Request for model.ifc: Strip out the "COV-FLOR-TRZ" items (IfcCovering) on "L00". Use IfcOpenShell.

First a look at what the model holds.

```python
import ifcopenshell
import ifcopenshell.util.element

model = ifcopenshell.open("model.ifc")
print(model.schema)
storey = next(s for s in model.by_type("IfcBuildingStorey") if s.Name == "L00")
coverings = [e for e in ifcopenshell.util.element.get_decomposition(storey) if e.is_a("IfcCovering")]
seen = {}
for e in coverings:
    element_type = ifcopenshell.util.element.get_type(e)
    name = element_type.Name if element_type not in (None, e) else None
    seen[name] = seen.get(name, 0) + 1
for name, count in sorted(seen.items(), key=str):
    print(count, "x", name)
```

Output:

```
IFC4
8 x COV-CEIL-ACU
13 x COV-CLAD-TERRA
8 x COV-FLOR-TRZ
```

```python
import ifcopenshell
import ifcopenshell.api.root
import ifcopenshell.util.element

model = ifcopenshell.open("model.ifc")

storey = next(s for s in model.by_type("IfcBuildingStorey") if s.Name == "L00")
coverings = [e for e in ifcopenshell.util.element.get_decomposition(storey) if e.is_a("IfcCovering")]
targets = [e for e in coverings if (t := ifcopenshell.util.element.get_type(e)) not in (None, e) and t.Name == "COV-FLOR-TRZ"]

for e in targets:
    ifcopenshell.api.root.remove_product(model, product=e)
print(len(targets), "removed")

model.write("model_edited.ifc")
```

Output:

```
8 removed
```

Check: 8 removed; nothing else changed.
